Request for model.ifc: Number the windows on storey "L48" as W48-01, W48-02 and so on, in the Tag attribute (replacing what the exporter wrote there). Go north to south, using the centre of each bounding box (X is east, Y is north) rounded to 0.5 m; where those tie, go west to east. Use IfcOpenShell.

First a look at what the model holds.

```python
import ifcopenshell
import ifcopenshell.util.element
import ifcopenshell.util.placement

model = ifcopenshell.open("model.ifc")
print(model.schema)
storey = next(s for s in model.by_type("IfcBuildingStorey") if s.Name == "L48")
windows = [e for e in ifcopenshell.util.element.get_decomposition(storey) if e.is_a("IfcWindow")]
for e in sorted(windows, key=lambda e: e.id()):
    origin = ifcopenshell.util.placement.get_local_placement(e.ObjectPlacement)[:3, 3]
    print(e.id(), e.Tag, e.Name, origin.round(2) + 0.0, sep=" | ")
```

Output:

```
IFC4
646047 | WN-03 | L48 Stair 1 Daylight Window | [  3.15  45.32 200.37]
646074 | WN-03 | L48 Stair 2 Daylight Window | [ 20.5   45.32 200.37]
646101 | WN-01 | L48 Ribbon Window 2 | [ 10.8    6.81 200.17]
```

```python
import ifcopenshell
import ifcopenshell.geom
import ifcopenshell.util.element
import ifcopenshell.util.shape

model = ifcopenshell.open("model.ifc")
settings = ifcopenshell.geom.settings()
settings.set("use-world-coords", True)


def centre(element):
    shape = ifcopenshell.geom.create_shape(settings, element)
    return ifcopenshell.util.shape.get_bbox_centroid(shape.geometry)


storey = next(s for s in model.by_type("IfcBuildingStorey") if s.Name == "L48")
windows = [e for e in ifcopenshell.util.element.get_decomposition(storey) if e.is_a("IfcWindow")]

# Insertion points can sit at a corner or the storey origin, so sort by the geometry (in metres).
centres = {e: centre(e) for e in windows}
windows.sort(key=lambda e: (-round(centres[e][1] / 0.5), centres[e][0]))

for i, e in enumerate(windows, start=1):
    number = f"W48-{i:02d}"
    e.Tag = number
    print(e.id(), number)

model.write("model_updated.ifc")
```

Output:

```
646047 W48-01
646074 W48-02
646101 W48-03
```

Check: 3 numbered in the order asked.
